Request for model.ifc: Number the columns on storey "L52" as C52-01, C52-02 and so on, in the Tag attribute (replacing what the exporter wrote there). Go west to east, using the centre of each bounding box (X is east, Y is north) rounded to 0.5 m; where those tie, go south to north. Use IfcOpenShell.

First a look at what the model holds.

```python
import ifcopenshell
import ifcopenshell.util.element
import ifcopenshell.util.placement

model = ifcopenshell.open("model.ifc")
print(model.schema)
storey = next(s for s in model.by_type("IfcBuildingStorey") if s.Name == "L52")
columns = [e for e in ifcopenshell.util.element.get_decomposition(storey) if e.is_a("IfcColumn")]
for e in sorted(columns, key=lambda e: e.id()):
    origin = ifcopenshell.util.placement.get_local_placement(e.ObjectPlacement)[:3, 3]
    print(e.id(), e.Tag, e.Name, origin.round(2) + 0.0, sep=" | ")
```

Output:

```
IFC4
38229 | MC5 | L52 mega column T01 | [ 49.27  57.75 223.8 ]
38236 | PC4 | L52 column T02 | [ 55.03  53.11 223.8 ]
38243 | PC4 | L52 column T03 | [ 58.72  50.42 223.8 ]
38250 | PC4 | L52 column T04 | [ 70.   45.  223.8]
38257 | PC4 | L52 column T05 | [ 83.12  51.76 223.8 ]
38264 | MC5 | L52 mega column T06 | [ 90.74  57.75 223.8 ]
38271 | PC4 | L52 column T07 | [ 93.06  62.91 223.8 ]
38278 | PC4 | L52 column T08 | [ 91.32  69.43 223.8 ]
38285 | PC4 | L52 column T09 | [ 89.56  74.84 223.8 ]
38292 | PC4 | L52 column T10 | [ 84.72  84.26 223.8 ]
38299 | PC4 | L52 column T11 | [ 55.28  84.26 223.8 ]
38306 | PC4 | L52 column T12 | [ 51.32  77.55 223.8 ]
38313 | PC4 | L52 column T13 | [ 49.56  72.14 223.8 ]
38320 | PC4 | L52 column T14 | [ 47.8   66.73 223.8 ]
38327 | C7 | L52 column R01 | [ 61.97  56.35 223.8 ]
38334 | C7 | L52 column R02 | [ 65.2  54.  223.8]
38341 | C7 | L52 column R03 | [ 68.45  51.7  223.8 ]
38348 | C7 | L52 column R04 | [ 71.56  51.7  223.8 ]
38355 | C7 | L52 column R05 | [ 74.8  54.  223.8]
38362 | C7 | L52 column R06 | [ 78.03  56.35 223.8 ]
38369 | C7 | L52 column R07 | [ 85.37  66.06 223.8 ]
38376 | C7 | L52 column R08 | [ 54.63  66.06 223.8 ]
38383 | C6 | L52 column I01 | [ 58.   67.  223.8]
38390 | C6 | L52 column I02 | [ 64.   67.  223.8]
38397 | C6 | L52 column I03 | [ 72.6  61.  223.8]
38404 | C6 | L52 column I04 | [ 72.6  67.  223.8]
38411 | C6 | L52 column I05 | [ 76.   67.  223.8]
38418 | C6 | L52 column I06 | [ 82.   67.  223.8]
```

```python
import ifcopenshell
import ifcopenshell.geom
import ifcopenshell.util.element
import ifcopenshell.util.shape

model = ifcopenshell.open("model.ifc")
settings = ifcopenshell.geom.settings()
settings.set("use-world-coords", True)


def centre(element):
    shape = ifcopenshell.geom.create_shape(settings, element)
    return ifcopenshell.util.shape.get_bbox_centroid(shape.geometry)


storey = next(s for s in model.by_type("IfcBuildingStorey") if s.Name == "L52")
columns = [e for e in ifcopenshell.util.element.get_decomposition(storey) if e.is_a("IfcColumn")]

# Insertion points can sit at a corner or the storey origin, so sort by the geometry (in metres).
centres = {e: centre(e) for e in columns}
columns.sort(key=lambda e: (round(centres[e][0] / 0.5), centres[e][1]))

for i, e in enumerate(columns, start=1):
    number = f"C52-{i:02d}"
    e.Tag = number
    print(e.id(), number)

model.write("model_edited.ifc")
```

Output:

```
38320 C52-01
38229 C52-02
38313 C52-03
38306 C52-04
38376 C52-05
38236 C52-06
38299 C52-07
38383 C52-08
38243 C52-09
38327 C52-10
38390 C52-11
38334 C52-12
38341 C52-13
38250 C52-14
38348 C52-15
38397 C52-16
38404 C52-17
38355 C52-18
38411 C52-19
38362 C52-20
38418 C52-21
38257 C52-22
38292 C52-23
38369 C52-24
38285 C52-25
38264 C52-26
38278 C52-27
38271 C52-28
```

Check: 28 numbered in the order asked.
